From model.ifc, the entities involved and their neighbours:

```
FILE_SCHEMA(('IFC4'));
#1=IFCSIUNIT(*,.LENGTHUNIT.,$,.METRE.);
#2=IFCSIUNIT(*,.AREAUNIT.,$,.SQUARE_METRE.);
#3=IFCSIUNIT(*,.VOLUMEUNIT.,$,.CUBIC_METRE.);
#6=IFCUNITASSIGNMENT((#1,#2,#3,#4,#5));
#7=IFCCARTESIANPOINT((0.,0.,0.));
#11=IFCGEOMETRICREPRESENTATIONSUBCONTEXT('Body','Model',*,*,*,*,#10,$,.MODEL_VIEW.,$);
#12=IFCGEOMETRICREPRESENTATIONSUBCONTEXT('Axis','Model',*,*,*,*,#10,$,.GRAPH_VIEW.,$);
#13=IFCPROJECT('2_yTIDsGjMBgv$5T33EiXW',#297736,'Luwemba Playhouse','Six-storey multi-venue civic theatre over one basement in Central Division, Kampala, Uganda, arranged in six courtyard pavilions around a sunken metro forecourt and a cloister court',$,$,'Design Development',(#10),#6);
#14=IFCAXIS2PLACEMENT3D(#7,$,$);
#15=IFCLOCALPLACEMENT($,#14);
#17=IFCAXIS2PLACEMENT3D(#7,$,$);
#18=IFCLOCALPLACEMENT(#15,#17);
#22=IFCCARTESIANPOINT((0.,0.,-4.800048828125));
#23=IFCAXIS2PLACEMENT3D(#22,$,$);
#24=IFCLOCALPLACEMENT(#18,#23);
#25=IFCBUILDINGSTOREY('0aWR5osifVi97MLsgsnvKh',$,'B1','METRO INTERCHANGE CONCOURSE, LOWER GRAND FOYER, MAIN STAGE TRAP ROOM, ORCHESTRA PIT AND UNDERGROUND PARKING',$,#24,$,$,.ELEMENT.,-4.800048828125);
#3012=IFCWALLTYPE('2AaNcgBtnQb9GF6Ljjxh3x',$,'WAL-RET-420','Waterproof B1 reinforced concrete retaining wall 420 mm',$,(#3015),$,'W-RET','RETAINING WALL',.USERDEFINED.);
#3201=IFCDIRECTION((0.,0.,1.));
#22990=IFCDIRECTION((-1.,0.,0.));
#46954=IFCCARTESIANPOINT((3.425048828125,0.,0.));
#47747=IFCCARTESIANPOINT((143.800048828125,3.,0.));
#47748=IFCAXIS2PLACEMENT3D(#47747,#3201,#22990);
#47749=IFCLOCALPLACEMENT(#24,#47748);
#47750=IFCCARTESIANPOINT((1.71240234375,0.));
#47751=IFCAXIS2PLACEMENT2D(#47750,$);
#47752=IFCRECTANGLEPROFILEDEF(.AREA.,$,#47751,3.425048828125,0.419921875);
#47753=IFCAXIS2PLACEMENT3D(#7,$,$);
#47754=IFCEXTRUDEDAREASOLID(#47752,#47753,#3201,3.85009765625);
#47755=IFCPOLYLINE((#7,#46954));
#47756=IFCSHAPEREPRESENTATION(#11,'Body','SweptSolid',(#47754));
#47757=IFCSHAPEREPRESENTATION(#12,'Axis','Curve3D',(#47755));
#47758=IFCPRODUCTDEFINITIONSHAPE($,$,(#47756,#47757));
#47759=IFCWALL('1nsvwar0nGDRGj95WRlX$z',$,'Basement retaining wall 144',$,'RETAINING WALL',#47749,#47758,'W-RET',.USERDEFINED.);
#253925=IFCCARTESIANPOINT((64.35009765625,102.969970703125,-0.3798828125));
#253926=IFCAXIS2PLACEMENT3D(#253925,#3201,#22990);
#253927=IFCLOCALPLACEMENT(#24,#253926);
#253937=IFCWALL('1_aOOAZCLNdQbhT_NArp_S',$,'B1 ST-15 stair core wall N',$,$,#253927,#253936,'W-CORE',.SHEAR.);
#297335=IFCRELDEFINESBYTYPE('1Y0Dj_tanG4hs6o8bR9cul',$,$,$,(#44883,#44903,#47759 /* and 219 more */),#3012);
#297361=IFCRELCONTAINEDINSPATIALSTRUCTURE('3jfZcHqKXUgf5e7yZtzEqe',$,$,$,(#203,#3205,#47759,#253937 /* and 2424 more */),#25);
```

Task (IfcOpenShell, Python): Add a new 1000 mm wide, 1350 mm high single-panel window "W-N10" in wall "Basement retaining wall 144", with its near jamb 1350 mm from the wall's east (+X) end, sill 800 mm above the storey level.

```python
import numpy as np
import ifcopenshell
import ifcopenshell.api.feature
import ifcopenshell.api.geometry
import ifcopenshell.api.root
import ifcopenshell.api.spatial
import ifcopenshell.geom
import ifcopenshell.util.element
import ifcopenshell.util.placement
import ifcopenshell.util.representation
import ifcopenshell.util.shape
import ifcopenshell.util.unit

model = ifcopenshell.open("model.ifc")
unit_scale = ifcopenshell.util.unit.calculate_unit_scale(model)
settings = ifcopenshell.geom.settings()


def volume(element):
    """Net volume in cubic metres, openings subtracted."""
    shape = ifcopenshell.geom.create_shape(settings, element)
    return ifcopenshell.util.shape.get_volume(shape.geometry)


wall = model.by_guid("1nsvwar0nGDRGj95WRlX$z")
storey = ifcopenshell.util.element.get_container(wall, ifc_class="IfcBuildingStorey")
context = ifcopenshell.util.representation.get_context(model, "Model", "Body", "MODEL_VIEW")
before = volume(wall)

width, height, from_end, sill = 1, 1.35, 1.35, 0.8  # metres

# The wall runs along its own X axis, and the end named is its -X end.
wall_shape = ifcopenshell.geom.create_shape(settings, wall)
x, y, z = ifcopenshell.util.shape.get_vertices(wall_shape.geometry).T
start = x.min() + from_end
face, thickness = float(y.min()), float(y.max() - y.min())
wall_matrix = ifcopenshell.util.placement.get_local_placement(wall.ObjectPlacement)
level = ifcopenshell.util.placement.get_local_placement(storey.ObjectPlacement)[2, 3]


def in_wall(x, y):
    """Placement at x, y metres in the wall's axes, at sill height."""
    matrix = wall_matrix.copy()
    matrix[:, 3] = wall_matrix @ np.array([x / unit_scale, y / unit_scale, 0.0, 1.0])
    matrix[2, 3] = level + sill / unit_scale
    return matrix


# Opening: a box that overshoots both wall faces by 50 mm.
opening = ifcopenshell.api.root.create_entity(model, ifc_class="IfcOpeningElement", predefined_type="OPENING")
box = ifcopenshell.api.geometry.add_wall_representation(
    model, context=context, length=width, height=height, thickness=thickness + 0.1
)
ifcopenshell.api.geometry.assign_representation(model, product=opening, representation=box)
ifcopenshell.api.geometry.edit_object_placement(model, product=opening, matrix=in_wall(start, face - 0.05), is_si=False)
ifcopenshell.api.feature.add_feature(model, feature=opening, element=wall)

window = ifcopenshell.api.root.create_entity(model, ifc_class="IfcWindow", name="W-N10", predefined_type="WINDOW")
window.OverallWidth, window.OverallHeight = width / unit_scale, height / unit_scale
window.PartitioningType = "SINGLE_PANEL"
body = ifcopenshell.api.geometry.add_window_representation(
    model,
    context=context,
    overall_width=window.OverallWidth,
    overall_height=window.OverallHeight,
    partition_type="SINGLE_PANEL",
)
ifcopenshell.api.geometry.assign_representation(model, product=window, representation=body)
ifcopenshell.api.spatial.assign_container(model, products=[window], relating_structure=storey)
ifcopenshell.api.feature.add_filling(model, opening=opening, element=window)

# Centre the window in the wall's thickness.
ifcopenshell.api.geometry.edit_object_placement(model, product=window, matrix=in_wall(start, face), is_si=False)
window_shape = ifcopenshell.geom.create_shape(settings, window)
depth = ifcopenshell.util.shape.get_vertices(window_shape.geometry)[:, 1]
offset = face + thickness / 2 - (depth.min() + depth.max()) / 2
ifcopenshell.api.geometry.edit_object_placement(model, product=window, matrix=in_wall(start, offset), is_si=False)

after = volume(wall)

print(f"wall volume {before:.3f} -> {after:.3f} m3")

model.write("model_rev.ifc")
```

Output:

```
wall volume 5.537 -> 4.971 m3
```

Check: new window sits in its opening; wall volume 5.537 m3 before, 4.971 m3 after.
